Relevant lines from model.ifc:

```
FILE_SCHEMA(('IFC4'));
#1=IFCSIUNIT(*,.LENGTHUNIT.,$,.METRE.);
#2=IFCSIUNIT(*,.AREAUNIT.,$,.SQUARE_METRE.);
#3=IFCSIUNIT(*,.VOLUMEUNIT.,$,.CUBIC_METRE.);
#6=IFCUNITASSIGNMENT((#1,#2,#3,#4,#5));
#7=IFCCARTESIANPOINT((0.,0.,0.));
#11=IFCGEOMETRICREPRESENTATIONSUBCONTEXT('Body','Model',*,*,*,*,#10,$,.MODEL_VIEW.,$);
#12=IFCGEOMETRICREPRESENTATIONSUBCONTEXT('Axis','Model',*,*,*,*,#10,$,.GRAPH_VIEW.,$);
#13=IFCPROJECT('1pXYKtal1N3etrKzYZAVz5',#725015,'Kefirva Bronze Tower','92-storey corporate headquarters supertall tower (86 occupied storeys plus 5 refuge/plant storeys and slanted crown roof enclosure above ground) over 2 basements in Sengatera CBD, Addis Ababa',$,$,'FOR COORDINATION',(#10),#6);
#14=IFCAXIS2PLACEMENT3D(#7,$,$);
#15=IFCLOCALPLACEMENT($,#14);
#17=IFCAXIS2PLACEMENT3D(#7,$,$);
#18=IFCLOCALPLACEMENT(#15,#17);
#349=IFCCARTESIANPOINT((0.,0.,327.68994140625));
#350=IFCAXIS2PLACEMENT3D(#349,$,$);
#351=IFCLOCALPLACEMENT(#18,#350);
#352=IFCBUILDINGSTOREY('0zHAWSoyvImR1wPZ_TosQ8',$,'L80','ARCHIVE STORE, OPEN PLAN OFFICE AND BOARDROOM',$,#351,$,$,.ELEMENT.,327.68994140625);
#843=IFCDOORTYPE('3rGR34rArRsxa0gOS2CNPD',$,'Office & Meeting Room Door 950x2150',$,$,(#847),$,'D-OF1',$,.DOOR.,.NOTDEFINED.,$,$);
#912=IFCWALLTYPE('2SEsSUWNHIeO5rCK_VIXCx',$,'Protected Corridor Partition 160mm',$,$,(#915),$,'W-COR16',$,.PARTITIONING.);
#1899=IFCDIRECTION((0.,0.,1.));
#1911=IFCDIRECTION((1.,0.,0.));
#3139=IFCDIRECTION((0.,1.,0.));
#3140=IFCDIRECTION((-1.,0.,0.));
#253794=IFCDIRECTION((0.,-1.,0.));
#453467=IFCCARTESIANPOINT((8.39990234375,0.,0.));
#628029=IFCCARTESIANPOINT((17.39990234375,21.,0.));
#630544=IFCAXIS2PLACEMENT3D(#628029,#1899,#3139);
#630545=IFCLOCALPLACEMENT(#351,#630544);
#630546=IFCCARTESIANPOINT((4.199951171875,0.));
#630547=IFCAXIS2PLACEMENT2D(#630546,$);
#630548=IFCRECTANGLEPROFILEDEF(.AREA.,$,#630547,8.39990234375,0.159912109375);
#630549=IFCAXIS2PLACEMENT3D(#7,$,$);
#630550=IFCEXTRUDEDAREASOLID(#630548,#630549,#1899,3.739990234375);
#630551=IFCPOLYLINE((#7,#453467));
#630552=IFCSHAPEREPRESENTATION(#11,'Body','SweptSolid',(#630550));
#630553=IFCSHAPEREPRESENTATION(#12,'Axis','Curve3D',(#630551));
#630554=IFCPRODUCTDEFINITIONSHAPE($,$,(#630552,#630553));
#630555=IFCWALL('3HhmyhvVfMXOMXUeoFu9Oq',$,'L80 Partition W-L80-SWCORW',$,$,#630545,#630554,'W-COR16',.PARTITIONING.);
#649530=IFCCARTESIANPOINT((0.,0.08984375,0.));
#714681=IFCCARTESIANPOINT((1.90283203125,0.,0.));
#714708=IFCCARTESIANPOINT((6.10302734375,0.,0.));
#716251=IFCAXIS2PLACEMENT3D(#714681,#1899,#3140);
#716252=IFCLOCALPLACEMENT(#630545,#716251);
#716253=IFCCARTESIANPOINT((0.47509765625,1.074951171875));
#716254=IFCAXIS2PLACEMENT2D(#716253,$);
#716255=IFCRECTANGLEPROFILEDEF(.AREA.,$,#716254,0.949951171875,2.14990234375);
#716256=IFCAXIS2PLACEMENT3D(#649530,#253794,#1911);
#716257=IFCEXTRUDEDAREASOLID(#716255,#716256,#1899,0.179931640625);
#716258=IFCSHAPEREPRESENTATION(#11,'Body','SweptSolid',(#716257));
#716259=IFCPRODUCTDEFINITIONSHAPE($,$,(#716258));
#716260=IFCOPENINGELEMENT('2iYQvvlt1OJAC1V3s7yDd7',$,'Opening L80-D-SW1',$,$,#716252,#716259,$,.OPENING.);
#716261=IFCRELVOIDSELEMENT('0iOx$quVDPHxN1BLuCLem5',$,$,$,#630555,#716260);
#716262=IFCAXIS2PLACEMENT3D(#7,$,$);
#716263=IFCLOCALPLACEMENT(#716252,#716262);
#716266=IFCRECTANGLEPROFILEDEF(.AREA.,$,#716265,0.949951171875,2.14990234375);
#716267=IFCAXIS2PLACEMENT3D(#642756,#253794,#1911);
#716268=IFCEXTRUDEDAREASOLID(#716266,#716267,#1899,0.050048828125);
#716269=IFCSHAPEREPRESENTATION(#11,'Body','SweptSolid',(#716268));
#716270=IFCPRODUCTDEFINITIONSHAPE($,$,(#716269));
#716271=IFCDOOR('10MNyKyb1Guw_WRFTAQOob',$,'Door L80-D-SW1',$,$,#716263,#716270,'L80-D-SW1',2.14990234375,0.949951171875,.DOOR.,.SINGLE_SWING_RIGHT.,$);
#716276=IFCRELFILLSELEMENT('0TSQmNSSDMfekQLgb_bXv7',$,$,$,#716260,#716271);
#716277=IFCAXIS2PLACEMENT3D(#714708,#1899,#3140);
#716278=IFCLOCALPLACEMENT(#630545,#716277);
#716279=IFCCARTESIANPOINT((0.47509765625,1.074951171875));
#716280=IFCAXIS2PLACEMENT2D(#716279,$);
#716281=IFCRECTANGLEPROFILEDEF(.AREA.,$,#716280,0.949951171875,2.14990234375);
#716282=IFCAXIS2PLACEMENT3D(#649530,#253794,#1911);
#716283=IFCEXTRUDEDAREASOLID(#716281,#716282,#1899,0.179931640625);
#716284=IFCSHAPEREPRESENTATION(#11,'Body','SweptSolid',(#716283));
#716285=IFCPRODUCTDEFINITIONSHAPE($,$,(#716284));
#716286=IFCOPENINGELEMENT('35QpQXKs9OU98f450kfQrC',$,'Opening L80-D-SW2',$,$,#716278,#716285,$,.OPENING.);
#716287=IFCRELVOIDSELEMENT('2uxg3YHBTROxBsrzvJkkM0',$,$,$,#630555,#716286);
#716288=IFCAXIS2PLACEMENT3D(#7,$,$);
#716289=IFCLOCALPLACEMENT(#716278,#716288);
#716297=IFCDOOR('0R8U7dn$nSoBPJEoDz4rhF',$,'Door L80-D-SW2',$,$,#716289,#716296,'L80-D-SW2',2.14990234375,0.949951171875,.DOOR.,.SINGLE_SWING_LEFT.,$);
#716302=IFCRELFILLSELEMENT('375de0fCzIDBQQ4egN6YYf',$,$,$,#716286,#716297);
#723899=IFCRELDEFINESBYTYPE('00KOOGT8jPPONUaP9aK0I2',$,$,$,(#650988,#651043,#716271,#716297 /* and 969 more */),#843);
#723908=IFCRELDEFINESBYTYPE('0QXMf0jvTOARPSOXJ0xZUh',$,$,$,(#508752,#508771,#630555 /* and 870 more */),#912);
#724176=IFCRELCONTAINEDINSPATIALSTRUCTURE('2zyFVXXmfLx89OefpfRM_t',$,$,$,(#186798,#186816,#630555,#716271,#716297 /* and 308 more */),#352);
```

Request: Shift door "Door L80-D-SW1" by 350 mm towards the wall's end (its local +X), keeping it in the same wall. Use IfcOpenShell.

```python
import ifcopenshell
import ifcopenshell.api.geometry
import ifcopenshell.util.placement
import ifcopenshell.util.unit

model = ifcopenshell.open("model.ifc")
unit_scale = ifcopenshell.util.unit.calculate_unit_scale(model)

door = model.by_guid("10MNyKyb1Guw_WRFTAQOob")
opening = door.FillsVoids[0].RelatingOpeningElement
wall = opening.VoidsElements[0].RelatingBuildingElement

wall_matrix = ifcopenshell.util.placement.get_local_placement(wall.ObjectPlacement)
shift = wall_matrix[:3, 0] * 0.35 / unit_scale
before = ifcopenshell.util.placement.get_local_placement(door.ObjectPlacement)[:3, 3].copy()

# The door is placed relative to its opening, so it follows when the opening moves.
matrix = ifcopenshell.util.placement.get_local_placement(opening.ObjectPlacement)
matrix[:3, 3] += shift
ifcopenshell.api.geometry.edit_object_placement(
    model, product=opening, matrix=matrix, is_si=False, should_transform_children=True
)

after = ifcopenshell.util.placement.get_local_placement(door.ObjectPlacement)[:3, 3]
print("door moved by", (after - before).round(3) + 0.0)

model.write("model_v2.ifc")
```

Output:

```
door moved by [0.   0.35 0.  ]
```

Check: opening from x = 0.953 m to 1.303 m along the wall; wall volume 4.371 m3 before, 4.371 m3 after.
